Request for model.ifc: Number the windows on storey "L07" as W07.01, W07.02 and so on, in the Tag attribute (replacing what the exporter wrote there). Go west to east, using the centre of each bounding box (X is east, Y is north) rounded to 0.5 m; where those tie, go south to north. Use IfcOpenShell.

First a look at what the model holds.

```python
import ifcopenshell
import ifcopenshell.util.element
import ifcopenshell.util.placement

model = ifcopenshell.open("model.ifc")
print(model.schema)
storey = next(s for s in model.by_type("IfcBuildingStorey") if s.Name == "L07")
windows = [e for e in ifcopenshell.util.element.get_decomposition(storey) if e.is_a("IfcWindow")]
for e in sorted(windows, key=lambda e: e.id()):
    origin = ifcopenshell.util.placement.get_local_placement(e.ObjectPlacement)[:3, 3]
    print(e.id(), e.Tag, e.Name, origin.round(2) + 0.0, sep=" | ")
```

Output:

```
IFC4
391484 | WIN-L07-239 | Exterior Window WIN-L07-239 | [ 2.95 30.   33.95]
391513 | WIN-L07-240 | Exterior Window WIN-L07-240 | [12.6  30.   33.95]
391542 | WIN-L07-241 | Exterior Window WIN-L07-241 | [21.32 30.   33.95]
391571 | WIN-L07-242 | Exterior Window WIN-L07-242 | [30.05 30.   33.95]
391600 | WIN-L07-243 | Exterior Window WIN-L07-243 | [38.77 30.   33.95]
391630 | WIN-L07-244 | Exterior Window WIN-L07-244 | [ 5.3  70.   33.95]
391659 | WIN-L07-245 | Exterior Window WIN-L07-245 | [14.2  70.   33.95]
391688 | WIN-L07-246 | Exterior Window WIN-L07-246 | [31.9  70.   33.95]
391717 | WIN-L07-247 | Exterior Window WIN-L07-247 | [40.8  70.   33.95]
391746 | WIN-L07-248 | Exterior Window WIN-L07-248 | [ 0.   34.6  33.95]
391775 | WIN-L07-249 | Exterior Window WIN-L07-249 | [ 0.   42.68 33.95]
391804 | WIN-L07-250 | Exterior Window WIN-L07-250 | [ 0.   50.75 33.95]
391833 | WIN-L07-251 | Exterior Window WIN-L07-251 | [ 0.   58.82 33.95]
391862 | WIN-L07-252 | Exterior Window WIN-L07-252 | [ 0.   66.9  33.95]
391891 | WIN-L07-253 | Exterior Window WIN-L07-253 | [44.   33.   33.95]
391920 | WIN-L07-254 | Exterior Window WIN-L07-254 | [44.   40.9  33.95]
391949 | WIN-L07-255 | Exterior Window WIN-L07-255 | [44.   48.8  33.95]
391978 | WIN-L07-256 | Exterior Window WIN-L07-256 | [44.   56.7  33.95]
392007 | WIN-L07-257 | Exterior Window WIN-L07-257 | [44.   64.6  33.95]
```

```python
import ifcopenshell
import ifcopenshell.geom
import ifcopenshell.util.element
import ifcopenshell.util.shape

model = ifcopenshell.open("model.ifc")
settings = ifcopenshell.geom.settings()
settings.set("use-world-coords", True)


def centre(element):
    shape = ifcopenshell.geom.create_shape(settings, element)
    return ifcopenshell.util.shape.get_bbox_centroid(shape.geometry)


storey = next(s for s in model.by_type("IfcBuildingStorey") if s.Name == "L07")
windows = [e for e in ifcopenshell.util.element.get_decomposition(storey) if e.is_a("IfcWindow")]

# Insertion points can sit at a corner or the storey origin, so sort by the geometry (in metres).
centres = {e: centre(e) for e in windows}
windows.sort(key=lambda e: (round(centres[e][0] / 0.5), centres[e][1]))

for i, e in enumerate(windows, start=1):
    number = f"W07.{i:02d}"
    e.Tag = number
    print(e.id(), number)

model.write("model_edited.ifc")
```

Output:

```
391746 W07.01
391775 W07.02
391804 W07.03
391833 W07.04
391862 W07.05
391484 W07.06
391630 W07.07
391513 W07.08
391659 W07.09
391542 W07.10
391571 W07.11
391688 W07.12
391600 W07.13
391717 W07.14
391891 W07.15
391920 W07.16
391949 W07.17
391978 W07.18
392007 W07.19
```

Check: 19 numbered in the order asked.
